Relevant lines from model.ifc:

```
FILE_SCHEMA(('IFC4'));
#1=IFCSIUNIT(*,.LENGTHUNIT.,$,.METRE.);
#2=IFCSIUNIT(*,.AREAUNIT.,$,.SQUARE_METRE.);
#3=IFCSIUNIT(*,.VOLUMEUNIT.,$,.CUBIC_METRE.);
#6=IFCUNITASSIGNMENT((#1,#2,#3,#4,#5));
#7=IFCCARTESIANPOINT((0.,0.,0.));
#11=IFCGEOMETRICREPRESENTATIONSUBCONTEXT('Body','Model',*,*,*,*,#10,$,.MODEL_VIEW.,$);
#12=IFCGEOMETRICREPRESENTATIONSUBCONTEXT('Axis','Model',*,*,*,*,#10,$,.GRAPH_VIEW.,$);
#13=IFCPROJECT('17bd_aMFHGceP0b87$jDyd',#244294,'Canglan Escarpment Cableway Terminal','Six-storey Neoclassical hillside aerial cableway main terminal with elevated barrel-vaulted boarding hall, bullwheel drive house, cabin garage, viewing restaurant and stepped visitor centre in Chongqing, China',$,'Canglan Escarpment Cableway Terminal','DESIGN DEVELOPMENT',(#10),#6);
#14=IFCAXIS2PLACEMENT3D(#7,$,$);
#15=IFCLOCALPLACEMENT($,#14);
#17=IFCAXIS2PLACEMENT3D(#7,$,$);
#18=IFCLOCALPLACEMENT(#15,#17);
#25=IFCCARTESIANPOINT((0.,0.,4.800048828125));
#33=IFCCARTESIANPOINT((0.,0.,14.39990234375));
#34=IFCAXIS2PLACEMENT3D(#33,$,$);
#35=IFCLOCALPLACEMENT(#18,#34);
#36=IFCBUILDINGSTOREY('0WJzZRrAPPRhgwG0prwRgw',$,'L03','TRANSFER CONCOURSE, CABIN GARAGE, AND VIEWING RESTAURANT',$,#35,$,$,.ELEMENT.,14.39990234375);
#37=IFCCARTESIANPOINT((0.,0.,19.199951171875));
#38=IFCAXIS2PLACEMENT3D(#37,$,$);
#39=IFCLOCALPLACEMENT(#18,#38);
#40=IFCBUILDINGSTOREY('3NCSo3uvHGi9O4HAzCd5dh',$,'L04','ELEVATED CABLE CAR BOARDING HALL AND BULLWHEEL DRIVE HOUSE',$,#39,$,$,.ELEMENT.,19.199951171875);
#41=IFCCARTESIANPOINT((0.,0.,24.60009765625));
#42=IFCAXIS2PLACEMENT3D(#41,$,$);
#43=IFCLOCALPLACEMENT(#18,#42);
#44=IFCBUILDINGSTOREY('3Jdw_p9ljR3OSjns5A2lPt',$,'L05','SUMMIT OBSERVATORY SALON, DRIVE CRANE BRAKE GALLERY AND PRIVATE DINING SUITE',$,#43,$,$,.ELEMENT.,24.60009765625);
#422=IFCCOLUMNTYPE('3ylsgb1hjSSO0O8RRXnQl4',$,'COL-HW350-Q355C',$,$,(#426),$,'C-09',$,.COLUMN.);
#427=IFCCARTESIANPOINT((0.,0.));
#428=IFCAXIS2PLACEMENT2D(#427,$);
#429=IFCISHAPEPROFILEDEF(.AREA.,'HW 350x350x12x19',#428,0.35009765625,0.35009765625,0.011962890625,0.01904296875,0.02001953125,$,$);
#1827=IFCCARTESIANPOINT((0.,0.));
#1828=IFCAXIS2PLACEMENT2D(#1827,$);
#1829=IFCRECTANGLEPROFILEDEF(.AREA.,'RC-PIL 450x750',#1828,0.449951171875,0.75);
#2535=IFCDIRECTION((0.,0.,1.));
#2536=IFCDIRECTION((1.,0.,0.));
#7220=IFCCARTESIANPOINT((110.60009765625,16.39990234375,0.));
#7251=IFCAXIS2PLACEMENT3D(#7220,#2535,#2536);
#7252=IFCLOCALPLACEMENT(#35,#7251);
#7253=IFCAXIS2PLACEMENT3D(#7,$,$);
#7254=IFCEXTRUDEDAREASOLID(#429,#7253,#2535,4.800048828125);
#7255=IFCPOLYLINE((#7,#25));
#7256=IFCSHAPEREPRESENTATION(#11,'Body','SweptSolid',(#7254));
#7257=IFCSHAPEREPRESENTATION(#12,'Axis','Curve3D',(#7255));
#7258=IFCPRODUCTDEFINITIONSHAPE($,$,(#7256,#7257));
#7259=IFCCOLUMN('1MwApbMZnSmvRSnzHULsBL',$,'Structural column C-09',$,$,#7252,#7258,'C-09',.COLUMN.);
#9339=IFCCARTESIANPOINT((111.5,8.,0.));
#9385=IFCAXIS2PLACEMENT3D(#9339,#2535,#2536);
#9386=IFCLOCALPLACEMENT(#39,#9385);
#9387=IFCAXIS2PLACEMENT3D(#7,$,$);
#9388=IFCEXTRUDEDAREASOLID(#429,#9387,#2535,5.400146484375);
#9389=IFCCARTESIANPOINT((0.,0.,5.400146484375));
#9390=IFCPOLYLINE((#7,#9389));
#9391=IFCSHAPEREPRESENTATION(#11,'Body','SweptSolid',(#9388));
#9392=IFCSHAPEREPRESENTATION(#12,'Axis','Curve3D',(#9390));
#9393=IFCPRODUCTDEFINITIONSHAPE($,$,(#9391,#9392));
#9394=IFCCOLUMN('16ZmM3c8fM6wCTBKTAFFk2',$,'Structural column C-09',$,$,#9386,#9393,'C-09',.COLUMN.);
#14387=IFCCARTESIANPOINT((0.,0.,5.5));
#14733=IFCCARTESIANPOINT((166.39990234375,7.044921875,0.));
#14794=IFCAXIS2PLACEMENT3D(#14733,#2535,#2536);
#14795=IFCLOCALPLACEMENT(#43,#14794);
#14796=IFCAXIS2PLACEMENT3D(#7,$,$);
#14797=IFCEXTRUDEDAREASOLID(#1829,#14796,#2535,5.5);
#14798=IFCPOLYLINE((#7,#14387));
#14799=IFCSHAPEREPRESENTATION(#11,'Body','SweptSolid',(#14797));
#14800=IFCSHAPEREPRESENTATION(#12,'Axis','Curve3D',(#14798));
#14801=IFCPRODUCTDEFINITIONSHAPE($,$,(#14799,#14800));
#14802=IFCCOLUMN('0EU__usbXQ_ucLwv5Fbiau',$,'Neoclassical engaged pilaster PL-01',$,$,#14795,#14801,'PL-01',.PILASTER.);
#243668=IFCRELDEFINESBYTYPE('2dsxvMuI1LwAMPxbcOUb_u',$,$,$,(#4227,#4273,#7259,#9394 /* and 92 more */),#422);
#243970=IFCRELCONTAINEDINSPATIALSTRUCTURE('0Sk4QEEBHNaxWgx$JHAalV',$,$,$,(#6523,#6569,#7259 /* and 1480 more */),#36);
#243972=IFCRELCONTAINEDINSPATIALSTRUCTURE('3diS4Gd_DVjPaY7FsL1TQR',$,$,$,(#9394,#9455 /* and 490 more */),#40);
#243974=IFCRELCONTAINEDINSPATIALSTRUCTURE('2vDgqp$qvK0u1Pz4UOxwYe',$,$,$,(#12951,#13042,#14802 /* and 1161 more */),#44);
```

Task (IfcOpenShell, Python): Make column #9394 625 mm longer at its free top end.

```python
import numpy as np
import ifcopenshell
import ifcopenshell.util.representation

model = ifcopenshell.open("model.ifc")

member = model.by_guid("16ZmM3c8fM6wCTBKTAFFk2")
change = 0.625

# The extrusion runs towards the end named, so only its depth changes.
body = ifcopenshell.util.representation.get_representation(member, "Model", "Body")
solid = body.Items[0]
old_length = solid.Depth
solid.Depth += change

# Move the axis end point with it.
axis = next(r for r in member.Representation.Representations if r.RepresentationIdentifier == "Axis").Items[0]
start, end = (np.array(p.Coordinates) for p in axis.Points)
end = end + (end - start) / np.linalg.norm(end - start) * change
point = model.createIfcCartesianPoint(end.tolist())
axis.Points = [axis.Points[0], point]

print(f"length {old_length:g} -> {solid.Depth:g}")

model.write("model_edited.ifc")
```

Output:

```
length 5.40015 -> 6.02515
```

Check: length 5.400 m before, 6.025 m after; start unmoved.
